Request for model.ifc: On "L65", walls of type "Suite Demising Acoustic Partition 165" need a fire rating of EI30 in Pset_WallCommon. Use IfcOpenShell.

First a look at what the model holds.

```python
import ifcopenshell
import ifcopenshell.util.element

model = ifcopenshell.open("model.ifc")
print(model.schema)
storey = next(s for s in model.by_type("IfcBuildingStorey") if s.Name == "L65")
walls = [e for e in ifcopenshell.util.element.get_decomposition(storey) if e.is_a("IfcWall")]
seen = {}
for e in walls:
    element_type = ifcopenshell.util.element.get_type(e)
    key = (element_type.Name if element_type != e and element_type else None, ifcopenshell.util.element.get_pset(e, "Pset_WallCommon", "FireRating"))
    seen[key] = seen.get(key, 0) + 1
for (name, value), count in sorted(seen.items(), key=str):
    print(count, "x", name, "|", value)
```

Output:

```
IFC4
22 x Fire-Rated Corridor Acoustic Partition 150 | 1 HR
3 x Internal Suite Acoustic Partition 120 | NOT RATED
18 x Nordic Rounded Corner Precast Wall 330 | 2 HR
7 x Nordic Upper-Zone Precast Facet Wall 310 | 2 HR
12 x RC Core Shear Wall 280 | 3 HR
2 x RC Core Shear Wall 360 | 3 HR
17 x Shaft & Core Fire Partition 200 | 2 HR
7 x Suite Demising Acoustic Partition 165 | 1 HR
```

```python
import ifcopenshell
import ifcopenshell.api.pset
import ifcopenshell.util.element

model = ifcopenshell.open("model.ifc")

storey = next(s for s in model.by_type("IfcBuildingStorey") if s.Name == "L65")
walls = [e for e in ifcopenshell.util.element.get_decomposition(storey) if e.is_a("IfcWall")]

count = 0
for e in walls:
    element_type = ifcopenshell.util.element.get_type(e)
    if element_type in (None, e) or element_type.Name != "Suite Demising Acoustic Partition 165":
        continue
    found = ifcopenshell.util.element.get_pset(e, "Pset_WallCommon", should_inherit=False)
    if found:
        pset = model.by_id(found["id"])
        if len(ifcopenshell.util.element.get_elements_by_pset(pset)) > 1:
            pset = ifcopenshell.api.pset.unshare_pset(model, products=[e], pset=pset)[0]
    else:
        pset = ifcopenshell.api.pset.add_pset(model, product=e, name="Pset_WallCommon")
    ifcopenshell.api.pset.edit_pset(model, pset=pset, properties={"FireRating": "EI30"})
    count += 1

print(count, "walls updated")

model.write("model_edited.ifc")
```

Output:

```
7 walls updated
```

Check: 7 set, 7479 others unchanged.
